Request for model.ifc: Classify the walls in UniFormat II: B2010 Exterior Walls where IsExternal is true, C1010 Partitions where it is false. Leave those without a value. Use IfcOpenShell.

First a look at what the model holds.

```python
import ifcopenshell
import ifcopenshell.util.element

model = ifcopenshell.open("model.ifc")
print(model.schema)
print("classifications:", [c.Name for c in model.by_type("IfcClassification")])
values = [ifcopenshell.util.element.get_pset(e, "Pset_WallCommon", "IsExternal") for e in model.by_type("IfcWall")]
for value in (True, False, None):
    print("IsExternal", value, values.count(value))
```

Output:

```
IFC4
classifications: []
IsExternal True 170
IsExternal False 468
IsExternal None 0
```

```python
import ifcopenshell
import ifcopenshell.api.classification
import ifcopenshell.util.element

model = ifcopenshell.open("model.ifc")

system = ifcopenshell.api.classification.add_classification(model, classification="UniFormat II")

walls = model.by_type("IfcWall")
external = {e: ifcopenshell.util.element.get_pset(e, "Pset_WallCommon", "IsExternal") for e in walls}
for flag, code, name in ((True, "B2010", "Exterior Walls"), (False, "C1010", "Partitions")):
    products = [e for e in walls if external[e] is flag]
    ifcopenshell.api.classification.add_reference(
        model, products=products, classification=system, identification=code, name=name
    )
    print(code, len(products))

model.write("model_v2.ifc")
```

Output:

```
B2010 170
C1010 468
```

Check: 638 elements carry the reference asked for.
